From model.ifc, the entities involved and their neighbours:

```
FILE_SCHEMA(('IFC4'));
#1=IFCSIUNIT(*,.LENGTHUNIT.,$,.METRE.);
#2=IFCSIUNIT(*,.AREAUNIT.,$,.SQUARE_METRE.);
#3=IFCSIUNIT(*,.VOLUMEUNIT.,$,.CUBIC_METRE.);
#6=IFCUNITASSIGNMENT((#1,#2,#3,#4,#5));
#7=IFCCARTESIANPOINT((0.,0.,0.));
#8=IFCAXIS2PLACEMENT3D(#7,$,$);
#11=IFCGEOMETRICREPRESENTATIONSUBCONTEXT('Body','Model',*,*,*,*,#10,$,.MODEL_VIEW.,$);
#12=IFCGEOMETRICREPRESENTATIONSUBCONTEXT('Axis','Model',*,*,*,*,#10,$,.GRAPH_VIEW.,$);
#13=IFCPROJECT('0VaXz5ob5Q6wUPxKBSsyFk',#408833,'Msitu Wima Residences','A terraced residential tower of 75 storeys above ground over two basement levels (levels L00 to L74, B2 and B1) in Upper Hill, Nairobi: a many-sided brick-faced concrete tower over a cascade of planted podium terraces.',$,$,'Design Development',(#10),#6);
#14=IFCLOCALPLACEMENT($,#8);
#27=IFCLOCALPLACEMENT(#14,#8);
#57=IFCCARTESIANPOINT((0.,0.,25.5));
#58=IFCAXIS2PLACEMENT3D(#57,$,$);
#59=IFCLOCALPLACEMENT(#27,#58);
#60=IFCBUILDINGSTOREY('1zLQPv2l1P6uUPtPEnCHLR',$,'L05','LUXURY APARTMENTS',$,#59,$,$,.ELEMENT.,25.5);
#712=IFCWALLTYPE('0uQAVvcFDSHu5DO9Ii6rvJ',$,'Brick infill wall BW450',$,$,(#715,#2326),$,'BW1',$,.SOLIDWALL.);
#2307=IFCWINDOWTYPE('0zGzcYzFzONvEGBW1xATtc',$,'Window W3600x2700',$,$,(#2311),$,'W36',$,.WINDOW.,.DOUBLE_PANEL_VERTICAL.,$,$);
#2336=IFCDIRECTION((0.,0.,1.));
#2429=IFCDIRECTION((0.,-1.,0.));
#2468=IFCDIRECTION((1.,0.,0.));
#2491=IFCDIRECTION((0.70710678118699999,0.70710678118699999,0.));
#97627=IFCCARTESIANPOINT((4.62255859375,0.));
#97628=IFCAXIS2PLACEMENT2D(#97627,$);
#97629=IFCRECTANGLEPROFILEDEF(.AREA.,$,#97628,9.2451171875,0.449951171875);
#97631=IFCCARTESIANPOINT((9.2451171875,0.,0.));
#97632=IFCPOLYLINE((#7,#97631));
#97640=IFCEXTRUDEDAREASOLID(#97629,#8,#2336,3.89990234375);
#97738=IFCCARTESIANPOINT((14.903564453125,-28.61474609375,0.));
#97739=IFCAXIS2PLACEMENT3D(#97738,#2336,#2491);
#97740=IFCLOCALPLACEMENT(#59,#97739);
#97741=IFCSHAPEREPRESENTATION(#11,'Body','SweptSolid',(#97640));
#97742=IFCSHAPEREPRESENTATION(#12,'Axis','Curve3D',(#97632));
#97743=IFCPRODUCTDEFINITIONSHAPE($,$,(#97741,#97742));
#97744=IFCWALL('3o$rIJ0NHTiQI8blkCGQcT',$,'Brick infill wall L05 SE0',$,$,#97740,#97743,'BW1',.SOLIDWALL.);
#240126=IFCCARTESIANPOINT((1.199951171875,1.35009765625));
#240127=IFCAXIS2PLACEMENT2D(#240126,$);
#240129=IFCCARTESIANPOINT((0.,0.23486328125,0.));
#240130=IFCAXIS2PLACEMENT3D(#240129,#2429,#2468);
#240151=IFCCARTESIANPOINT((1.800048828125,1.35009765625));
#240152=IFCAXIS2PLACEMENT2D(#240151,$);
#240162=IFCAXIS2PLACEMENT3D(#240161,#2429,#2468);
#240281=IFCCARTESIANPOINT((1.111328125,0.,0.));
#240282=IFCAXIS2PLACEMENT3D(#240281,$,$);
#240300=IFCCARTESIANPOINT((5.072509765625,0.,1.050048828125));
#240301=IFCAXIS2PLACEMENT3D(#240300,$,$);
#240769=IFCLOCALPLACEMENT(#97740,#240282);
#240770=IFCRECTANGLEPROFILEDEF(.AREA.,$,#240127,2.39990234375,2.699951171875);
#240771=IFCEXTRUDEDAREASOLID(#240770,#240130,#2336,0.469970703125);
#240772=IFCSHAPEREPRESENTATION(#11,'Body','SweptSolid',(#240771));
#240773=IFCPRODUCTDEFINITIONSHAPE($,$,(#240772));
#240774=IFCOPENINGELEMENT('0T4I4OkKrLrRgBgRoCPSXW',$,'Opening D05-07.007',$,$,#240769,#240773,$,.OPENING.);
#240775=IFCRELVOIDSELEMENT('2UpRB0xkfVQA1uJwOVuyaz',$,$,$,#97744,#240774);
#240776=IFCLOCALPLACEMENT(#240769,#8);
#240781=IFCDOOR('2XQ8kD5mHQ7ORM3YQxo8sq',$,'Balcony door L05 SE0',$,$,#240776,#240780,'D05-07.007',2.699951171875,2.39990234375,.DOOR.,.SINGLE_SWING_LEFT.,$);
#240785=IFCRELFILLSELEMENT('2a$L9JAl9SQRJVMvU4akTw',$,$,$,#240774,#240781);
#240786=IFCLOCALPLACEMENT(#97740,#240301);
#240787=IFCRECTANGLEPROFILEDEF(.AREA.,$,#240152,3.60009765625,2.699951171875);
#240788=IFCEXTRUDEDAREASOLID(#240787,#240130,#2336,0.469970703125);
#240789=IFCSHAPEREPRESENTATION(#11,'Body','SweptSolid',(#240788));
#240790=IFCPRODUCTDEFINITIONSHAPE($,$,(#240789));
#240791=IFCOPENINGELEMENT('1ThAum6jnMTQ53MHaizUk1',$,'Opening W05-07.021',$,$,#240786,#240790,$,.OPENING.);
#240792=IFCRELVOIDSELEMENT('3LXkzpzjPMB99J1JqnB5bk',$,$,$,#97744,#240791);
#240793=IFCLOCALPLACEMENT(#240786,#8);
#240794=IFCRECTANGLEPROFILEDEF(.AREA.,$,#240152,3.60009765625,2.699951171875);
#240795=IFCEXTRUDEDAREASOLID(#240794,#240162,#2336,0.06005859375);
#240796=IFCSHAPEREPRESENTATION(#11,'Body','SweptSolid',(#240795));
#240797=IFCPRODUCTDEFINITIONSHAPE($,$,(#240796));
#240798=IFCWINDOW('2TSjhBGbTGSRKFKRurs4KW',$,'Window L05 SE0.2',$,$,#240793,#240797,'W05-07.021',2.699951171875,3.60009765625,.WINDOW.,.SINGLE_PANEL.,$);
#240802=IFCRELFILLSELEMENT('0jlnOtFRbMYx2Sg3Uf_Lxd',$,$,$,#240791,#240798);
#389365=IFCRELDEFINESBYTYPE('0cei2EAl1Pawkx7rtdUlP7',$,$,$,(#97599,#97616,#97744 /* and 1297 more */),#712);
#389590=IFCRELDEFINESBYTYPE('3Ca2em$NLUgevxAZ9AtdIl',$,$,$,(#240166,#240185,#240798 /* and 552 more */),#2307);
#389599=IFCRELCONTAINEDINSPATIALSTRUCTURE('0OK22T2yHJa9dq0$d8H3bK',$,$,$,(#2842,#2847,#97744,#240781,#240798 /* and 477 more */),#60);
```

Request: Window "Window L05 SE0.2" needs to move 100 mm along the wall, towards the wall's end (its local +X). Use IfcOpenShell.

```python
import ifcopenshell
import ifcopenshell.api.geometry
import ifcopenshell.util.placement

model = ifcopenshell.open("model.ifc")

window = model.by_id(240798)
opening = window.FillsVoids[0].RelatingOpeningElement
wall = opening.VoidsElements[0].RelatingBuildingElement

wall_matrix = ifcopenshell.util.placement.get_local_placement(wall.ObjectPlacement)
shift = wall_matrix[:3, 0] * 0.1
before = ifcopenshell.util.placement.get_local_placement(window.ObjectPlacement)[:3, 3].copy()

# The window is placed relative to its opening, so it follows when the opening moves.
matrix = ifcopenshell.util.placement.get_local_placement(opening.ObjectPlacement)
matrix[:3, 3] += shift
ifcopenshell.api.geometry.edit_object_placement(
    model, product=opening, matrix=matrix, is_si=False, should_transform_children=True
)

after = ifcopenshell.util.placement.get_local_placement(window.ObjectPlacement)[:3, 3]
print("window moved by", (after - before).round(3) + 0.0)

model.write("model_updated.ifc")
```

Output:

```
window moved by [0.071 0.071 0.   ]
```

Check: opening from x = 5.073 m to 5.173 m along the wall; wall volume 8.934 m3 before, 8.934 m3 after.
